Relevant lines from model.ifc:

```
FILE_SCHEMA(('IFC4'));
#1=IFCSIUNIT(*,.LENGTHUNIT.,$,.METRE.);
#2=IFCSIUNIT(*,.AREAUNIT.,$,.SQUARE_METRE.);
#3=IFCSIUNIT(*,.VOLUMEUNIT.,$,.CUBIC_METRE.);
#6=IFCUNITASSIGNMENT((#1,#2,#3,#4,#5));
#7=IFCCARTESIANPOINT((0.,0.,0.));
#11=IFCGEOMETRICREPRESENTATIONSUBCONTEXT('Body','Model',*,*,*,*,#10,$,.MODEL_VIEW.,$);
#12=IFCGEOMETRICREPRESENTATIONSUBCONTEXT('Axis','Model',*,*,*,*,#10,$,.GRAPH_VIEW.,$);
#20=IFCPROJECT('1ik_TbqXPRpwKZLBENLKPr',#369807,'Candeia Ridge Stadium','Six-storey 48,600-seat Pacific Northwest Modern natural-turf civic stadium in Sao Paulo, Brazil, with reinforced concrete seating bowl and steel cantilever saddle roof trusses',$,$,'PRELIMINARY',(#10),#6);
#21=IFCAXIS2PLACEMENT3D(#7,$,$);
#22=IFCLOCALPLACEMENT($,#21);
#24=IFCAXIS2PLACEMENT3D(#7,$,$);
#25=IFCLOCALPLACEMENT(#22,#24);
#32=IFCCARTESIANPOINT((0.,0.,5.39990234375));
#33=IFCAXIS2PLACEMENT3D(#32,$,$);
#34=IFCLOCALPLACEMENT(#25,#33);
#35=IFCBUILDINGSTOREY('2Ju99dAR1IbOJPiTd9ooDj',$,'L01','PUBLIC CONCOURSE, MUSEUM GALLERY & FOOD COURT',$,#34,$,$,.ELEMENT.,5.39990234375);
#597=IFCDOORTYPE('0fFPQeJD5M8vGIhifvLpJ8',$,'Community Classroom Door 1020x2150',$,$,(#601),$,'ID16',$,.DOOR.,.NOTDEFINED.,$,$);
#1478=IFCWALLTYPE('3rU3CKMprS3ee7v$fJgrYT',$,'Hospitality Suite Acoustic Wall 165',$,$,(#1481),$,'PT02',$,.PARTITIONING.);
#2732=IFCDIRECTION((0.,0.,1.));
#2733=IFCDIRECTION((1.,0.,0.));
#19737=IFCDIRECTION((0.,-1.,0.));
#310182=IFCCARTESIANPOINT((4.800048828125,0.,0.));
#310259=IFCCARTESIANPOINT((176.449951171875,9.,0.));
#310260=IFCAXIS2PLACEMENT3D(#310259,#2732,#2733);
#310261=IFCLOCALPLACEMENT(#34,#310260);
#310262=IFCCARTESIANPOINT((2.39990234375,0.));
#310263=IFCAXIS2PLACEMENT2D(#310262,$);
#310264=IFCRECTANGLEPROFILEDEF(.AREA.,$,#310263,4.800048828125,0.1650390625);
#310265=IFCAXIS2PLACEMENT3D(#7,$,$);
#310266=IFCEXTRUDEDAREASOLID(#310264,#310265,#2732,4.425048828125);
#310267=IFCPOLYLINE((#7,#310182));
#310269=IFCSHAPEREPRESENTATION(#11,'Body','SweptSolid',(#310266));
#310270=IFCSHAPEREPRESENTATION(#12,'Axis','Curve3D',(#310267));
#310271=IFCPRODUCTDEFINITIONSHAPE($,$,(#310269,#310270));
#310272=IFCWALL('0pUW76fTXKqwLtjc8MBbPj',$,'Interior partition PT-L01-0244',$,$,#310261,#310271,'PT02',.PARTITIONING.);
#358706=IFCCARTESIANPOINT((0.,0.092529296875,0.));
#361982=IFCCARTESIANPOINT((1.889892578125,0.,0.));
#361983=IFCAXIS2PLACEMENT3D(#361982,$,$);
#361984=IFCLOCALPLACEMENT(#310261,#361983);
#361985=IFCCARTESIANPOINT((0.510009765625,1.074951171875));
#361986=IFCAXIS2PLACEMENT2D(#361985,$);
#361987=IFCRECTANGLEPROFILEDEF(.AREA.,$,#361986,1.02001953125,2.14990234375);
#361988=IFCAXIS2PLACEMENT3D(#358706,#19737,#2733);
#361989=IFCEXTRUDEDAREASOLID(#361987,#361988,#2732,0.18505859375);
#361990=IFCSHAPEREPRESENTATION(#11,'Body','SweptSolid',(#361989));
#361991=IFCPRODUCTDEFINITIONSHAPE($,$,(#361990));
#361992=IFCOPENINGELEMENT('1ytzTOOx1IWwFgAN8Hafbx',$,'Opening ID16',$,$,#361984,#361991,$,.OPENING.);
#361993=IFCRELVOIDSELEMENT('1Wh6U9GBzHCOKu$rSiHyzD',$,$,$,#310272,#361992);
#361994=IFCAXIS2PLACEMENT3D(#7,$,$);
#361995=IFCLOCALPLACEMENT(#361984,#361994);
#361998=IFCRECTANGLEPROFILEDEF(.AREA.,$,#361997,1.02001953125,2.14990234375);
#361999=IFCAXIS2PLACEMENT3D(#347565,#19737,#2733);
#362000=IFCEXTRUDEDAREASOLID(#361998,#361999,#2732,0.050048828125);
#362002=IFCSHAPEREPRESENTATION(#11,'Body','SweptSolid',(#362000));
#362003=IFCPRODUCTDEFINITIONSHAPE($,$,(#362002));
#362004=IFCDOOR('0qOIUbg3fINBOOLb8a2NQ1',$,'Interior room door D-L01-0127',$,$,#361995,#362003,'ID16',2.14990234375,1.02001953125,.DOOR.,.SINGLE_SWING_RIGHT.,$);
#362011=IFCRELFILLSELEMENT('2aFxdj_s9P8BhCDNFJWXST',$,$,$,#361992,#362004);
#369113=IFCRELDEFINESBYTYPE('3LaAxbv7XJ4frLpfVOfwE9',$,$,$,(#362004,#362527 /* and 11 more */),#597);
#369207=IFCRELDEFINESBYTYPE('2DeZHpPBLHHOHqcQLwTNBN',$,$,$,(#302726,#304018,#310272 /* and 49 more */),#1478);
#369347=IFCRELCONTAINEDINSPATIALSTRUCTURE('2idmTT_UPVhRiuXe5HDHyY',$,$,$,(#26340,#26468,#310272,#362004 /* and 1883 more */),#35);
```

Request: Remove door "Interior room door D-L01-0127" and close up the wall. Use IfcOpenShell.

```python
import ifcopenshell
import ifcopenshell.api.feature
import ifcopenshell.api.root
import ifcopenshell.geom
import ifcopenshell.util.shape

model = ifcopenshell.open("model.ifc")
settings = ifcopenshell.geom.settings()


def volume(element):
    """Net volume in cubic metres, openings subtracted."""
    shape = ifcopenshell.geom.create_shape(settings, element)
    return ifcopenshell.util.shape.get_volume(shape.geometry)


door = model.by_id(362004)
opening = door.FillsVoids[0].RelatingOpeningElement
wall = opening.VoidsElements[0].RelatingBuildingElement
before = volume(wall)

ifcopenshell.api.root.remove_product(model, product=door)
ifcopenshell.api.feature.remove_feature(model, feature=opening)

after = volume(wall)

print(f"wall volume {before:.3f} -> {after:.3f} m3")

model.write("model_updated.ifc")
```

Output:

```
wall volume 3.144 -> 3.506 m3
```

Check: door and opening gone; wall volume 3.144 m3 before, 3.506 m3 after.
